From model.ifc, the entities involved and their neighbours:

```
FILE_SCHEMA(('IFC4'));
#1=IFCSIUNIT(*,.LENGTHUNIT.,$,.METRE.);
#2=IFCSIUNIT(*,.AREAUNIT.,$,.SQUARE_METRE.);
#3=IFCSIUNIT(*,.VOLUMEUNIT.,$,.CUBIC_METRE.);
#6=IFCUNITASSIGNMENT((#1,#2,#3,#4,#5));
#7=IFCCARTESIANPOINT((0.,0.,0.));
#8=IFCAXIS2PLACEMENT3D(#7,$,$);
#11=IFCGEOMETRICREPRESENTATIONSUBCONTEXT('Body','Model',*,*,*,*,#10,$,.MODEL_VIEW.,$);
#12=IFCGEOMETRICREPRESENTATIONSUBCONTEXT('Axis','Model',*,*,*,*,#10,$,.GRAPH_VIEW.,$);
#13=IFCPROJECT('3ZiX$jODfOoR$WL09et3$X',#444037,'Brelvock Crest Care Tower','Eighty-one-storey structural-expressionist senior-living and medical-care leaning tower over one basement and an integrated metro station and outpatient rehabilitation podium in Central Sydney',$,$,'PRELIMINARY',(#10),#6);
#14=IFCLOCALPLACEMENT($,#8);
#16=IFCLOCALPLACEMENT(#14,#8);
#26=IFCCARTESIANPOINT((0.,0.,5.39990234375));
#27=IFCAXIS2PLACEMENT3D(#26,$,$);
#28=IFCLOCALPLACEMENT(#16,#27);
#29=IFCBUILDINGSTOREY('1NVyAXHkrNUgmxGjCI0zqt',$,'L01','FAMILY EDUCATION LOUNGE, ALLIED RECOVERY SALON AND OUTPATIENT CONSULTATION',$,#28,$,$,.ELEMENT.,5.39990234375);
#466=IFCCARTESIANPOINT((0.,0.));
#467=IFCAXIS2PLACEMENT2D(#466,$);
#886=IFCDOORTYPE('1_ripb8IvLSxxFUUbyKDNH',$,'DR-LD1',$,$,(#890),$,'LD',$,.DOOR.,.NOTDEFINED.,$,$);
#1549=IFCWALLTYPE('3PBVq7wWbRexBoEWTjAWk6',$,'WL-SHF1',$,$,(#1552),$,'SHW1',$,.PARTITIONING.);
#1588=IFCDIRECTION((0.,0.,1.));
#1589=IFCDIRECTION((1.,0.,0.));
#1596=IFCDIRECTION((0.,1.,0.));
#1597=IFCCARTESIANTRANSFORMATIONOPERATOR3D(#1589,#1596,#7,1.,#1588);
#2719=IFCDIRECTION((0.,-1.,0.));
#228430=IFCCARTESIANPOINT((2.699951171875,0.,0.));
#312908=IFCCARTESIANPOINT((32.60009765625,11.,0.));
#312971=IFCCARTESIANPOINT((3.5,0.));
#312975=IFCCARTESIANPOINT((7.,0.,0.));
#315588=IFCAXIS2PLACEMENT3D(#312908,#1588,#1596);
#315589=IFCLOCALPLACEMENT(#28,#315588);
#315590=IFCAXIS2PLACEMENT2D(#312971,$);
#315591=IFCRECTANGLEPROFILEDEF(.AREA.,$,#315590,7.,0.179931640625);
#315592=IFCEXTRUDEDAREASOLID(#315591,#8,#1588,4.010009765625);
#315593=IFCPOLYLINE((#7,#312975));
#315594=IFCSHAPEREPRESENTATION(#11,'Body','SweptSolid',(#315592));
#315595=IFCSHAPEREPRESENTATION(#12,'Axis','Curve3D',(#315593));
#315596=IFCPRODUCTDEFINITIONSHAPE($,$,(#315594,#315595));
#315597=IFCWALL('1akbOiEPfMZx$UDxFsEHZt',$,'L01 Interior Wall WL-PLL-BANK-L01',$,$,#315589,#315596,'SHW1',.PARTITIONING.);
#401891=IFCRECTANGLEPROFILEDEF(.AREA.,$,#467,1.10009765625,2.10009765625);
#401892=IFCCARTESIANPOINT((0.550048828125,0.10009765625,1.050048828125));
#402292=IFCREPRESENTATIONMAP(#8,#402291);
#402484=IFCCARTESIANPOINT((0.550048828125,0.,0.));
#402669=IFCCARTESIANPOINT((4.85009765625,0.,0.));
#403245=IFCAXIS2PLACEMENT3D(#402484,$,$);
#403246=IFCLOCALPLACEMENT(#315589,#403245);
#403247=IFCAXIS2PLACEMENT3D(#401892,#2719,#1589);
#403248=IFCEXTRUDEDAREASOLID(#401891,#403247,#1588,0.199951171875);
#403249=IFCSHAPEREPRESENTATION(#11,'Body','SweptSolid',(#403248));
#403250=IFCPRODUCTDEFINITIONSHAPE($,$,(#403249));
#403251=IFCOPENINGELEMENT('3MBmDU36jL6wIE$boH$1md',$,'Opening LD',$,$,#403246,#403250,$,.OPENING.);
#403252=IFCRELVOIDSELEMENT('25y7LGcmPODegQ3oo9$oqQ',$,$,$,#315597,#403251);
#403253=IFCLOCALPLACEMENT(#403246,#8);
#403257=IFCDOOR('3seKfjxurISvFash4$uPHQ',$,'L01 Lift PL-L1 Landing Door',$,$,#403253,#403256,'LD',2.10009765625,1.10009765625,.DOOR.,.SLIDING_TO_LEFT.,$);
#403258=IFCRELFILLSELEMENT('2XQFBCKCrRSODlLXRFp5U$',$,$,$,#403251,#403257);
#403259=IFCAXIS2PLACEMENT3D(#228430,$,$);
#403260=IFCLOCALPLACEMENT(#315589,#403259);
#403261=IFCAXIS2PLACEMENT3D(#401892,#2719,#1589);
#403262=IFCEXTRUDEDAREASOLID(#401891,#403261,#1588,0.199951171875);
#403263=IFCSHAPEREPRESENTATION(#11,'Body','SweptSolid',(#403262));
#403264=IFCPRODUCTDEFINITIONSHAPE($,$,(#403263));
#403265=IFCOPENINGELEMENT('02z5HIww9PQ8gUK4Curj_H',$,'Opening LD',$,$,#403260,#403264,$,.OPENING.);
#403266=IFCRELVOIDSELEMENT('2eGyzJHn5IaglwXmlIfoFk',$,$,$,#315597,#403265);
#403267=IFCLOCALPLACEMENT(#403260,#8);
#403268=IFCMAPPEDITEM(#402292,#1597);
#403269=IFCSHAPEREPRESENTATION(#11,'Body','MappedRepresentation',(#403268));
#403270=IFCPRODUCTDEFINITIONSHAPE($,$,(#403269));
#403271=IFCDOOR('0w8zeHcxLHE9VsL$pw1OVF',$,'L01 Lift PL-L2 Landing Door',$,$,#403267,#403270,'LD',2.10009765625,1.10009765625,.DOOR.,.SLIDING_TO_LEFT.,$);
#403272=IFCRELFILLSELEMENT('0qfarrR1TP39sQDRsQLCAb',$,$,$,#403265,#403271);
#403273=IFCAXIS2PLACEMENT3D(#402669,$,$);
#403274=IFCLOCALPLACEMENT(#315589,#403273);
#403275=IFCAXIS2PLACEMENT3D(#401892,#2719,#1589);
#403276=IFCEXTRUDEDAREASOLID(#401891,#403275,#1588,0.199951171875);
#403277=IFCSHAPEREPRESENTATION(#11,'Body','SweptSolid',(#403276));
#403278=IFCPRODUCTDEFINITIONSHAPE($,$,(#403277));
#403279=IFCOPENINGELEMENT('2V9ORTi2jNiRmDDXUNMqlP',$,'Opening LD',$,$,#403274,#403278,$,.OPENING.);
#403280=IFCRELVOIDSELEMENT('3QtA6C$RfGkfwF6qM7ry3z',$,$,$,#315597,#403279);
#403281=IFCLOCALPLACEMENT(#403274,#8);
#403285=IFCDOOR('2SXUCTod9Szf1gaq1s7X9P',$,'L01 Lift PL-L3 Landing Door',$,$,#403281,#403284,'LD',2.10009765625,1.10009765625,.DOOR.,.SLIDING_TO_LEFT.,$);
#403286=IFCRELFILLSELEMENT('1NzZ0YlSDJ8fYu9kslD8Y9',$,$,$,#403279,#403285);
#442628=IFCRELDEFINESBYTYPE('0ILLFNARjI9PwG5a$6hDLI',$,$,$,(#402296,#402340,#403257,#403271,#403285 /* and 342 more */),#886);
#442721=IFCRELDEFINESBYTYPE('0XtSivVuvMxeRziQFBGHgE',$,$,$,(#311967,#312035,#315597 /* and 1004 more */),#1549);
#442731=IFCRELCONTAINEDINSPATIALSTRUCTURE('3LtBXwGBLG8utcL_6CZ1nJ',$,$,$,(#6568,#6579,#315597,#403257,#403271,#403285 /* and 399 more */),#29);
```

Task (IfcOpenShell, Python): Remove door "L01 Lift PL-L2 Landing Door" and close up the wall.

```python
import ifcopenshell
import ifcopenshell.api.feature
import ifcopenshell.api.root
import ifcopenshell.geom
import ifcopenshell.util.shape

model = ifcopenshell.open("model.ifc")
settings = ifcopenshell.geom.settings()


def volume(element):
    """Net volume in cubic metres, openings subtracted."""
    shape = ifcopenshell.geom.create_shape(settings, element)
    return ifcopenshell.util.shape.get_volume(shape.geometry)


door = model.by_guid("0w8zeHcxLHE9VsL$pw1OVF")
opening = door.FillsVoids[0].RelatingOpeningElement
wall = opening.VoidsElements[0].RelatingBuildingElement
before = volume(wall)

ifcopenshell.api.root.remove_product(model, product=door)
ifcopenshell.api.feature.remove_feature(model, feature=opening)

after = volume(wall)

print(f"wall volume {before:.3f} -> {after:.3f} m3")

model.write("model-out.ifc")
```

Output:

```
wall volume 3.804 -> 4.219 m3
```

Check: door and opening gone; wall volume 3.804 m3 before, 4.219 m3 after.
